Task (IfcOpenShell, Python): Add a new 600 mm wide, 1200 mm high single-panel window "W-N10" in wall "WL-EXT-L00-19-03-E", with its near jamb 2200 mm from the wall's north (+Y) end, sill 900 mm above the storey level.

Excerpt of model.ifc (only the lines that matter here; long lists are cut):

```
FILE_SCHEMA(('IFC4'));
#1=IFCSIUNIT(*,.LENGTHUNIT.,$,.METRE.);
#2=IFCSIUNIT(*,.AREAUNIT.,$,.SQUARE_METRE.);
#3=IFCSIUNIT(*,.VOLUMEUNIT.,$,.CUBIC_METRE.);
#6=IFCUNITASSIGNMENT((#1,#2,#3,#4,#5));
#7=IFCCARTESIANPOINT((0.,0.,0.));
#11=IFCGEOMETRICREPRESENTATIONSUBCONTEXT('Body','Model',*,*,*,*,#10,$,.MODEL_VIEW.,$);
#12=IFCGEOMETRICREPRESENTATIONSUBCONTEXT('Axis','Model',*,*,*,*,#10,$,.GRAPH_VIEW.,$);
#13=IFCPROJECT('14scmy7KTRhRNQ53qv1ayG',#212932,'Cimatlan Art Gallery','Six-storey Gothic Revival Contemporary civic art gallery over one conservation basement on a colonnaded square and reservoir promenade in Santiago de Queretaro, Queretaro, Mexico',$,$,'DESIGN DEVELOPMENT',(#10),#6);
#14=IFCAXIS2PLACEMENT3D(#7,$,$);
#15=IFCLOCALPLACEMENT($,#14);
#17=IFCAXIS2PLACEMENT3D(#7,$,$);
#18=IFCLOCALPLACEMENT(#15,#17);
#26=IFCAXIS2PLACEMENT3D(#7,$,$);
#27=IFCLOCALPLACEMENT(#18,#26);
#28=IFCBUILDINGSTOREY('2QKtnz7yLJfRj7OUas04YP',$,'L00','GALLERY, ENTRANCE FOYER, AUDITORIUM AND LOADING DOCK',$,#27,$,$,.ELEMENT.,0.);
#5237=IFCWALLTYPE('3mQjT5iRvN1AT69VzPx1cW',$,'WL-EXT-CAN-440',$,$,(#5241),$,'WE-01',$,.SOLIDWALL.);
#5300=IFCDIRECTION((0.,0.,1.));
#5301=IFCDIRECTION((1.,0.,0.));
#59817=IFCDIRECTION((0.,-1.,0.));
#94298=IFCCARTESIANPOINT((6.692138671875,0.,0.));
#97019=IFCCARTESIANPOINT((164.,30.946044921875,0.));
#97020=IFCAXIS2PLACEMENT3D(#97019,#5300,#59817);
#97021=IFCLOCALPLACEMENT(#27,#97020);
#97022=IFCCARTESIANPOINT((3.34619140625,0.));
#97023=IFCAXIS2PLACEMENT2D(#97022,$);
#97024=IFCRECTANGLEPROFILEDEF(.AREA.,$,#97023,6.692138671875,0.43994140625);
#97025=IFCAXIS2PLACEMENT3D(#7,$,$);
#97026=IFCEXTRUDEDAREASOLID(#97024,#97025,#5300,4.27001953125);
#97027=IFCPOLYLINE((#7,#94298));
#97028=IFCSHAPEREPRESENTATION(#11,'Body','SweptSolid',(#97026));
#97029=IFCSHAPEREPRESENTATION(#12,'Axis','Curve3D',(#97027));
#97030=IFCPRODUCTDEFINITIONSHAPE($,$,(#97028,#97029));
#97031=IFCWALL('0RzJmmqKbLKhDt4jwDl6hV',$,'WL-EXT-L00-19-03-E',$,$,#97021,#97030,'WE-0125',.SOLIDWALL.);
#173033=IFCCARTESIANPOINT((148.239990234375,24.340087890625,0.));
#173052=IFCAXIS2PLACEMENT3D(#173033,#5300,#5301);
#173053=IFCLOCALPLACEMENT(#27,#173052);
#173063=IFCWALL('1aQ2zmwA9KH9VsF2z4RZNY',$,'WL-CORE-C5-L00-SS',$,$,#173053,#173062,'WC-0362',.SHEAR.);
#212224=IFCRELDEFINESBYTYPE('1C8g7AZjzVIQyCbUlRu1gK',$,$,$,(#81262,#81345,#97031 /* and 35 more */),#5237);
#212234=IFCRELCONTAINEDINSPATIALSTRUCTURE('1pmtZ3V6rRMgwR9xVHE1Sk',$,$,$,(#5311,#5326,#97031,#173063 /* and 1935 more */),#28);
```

```python
import numpy as np
import ifcopenshell
import ifcopenshell.api.feature
import ifcopenshell.api.geometry
import ifcopenshell.api.root
import ifcopenshell.api.spatial
import ifcopenshell.geom
import ifcopenshell.util.element
import ifcopenshell.util.placement
import ifcopenshell.util.representation
import ifcopenshell.util.shape
import ifcopenshell.util.unit

model = ifcopenshell.open("model.ifc")
unit_scale = ifcopenshell.util.unit.calculate_unit_scale(model)
settings = ifcopenshell.geom.settings()


def volume(element):
    """Net volume in cubic metres, openings subtracted."""
    shape = ifcopenshell.geom.create_shape(settings, element)
    return ifcopenshell.util.shape.get_volume(shape.geometry)


wall = model.by_guid("0RzJmmqKbLKhDt4jwDl6hV")
storey = ifcopenshell.util.element.get_container(wall, ifc_class="IfcBuildingStorey")
context = ifcopenshell.util.representation.get_context(model, "Model", "Body", "MODEL_VIEW")
before = volume(wall)

width, height, from_end, sill = 0.6, 1.2, 2.2, 0.9  # metres

# The wall runs along its own X axis, and the end named is its -X end.
wall_shape = ifcopenshell.geom.create_shape(settings, wall)
x, y, z = ifcopenshell.util.shape.get_vertices(wall_shape.geometry).T
start = x.min() + from_end
face, thickness = float(y.min()), float(y.max() - y.min())
wall_matrix = ifcopenshell.util.placement.get_local_placement(wall.ObjectPlacement)
level = ifcopenshell.util.placement.get_local_placement(storey.ObjectPlacement)[2, 3]


def in_wall(x, y):
    """Placement at x, y metres in the wall's axes, at sill height."""
    matrix = wall_matrix.copy()
    matrix[:, 3] = wall_matrix @ np.array([x / unit_scale, y / unit_scale, 0.0, 1.0])
    matrix[2, 3] = level + sill / unit_scale
    return matrix


# Opening: a box that overshoots both wall faces by 50 mm.
opening = ifcopenshell.api.root.create_entity(model, ifc_class="IfcOpeningElement", predefined_type="OPENING")
box = ifcopenshell.api.geometry.add_wall_representation(
    model, context=context, length=width, height=height, thickness=thickness + 0.1
)
ifcopenshell.api.geometry.assign_representation(model, product=opening, representation=box)
ifcopenshell.api.geometry.edit_object_placement(model, product=opening, matrix=in_wall(start, face - 0.05), is_si=False)
ifcopenshell.api.feature.add_feature(model, feature=opening, element=wall)

window = ifcopenshell.api.root.create_entity(model, ifc_class="IfcWindow", name="W-N10", predefined_type="WINDOW")
window.OverallWidth, window.OverallHeight = width / unit_scale, height / unit_scale
window.PartitioningType = "SINGLE_PANEL"
body = ifcopenshell.api.geometry.add_window_representation(
    model,
    context=context,
    overall_width=window.OverallWidth,
    overall_height=window.OverallHeight,
    partition_type="SINGLE_PANEL",
)
ifcopenshell.api.geometry.assign_representation(model, product=window, representation=body)
ifcopenshell.api.spatial.assign_container(model, products=[window], relating_structure=storey)
ifcopenshell.api.feature.add_filling(model, opening=opening, element=window)

# Centre the window in the wall's thickness.
ifcopenshell.api.geometry.edit_object_placement(model, product=window, matrix=in_wall(start, face), is_si=False)
window_shape = ifcopenshell.geom.create_shape(settings, window)
depth = ifcopenshell.util.shape.get_vertices(window_shape.geometry)[:, 1]
offset = face + thickness / 2 - (depth.min() + depth.max()) / 2
ifcopenshell.api.geometry.edit_object_placement(model, product=window, matrix=in_wall(start, offset), is_si=False)

after = volume(wall)

print(f"wall volume {before:.3f} -> {after:.3f} m3")

model.write("model_v2.ifc")
```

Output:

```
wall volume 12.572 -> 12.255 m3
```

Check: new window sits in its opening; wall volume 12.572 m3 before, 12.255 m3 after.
